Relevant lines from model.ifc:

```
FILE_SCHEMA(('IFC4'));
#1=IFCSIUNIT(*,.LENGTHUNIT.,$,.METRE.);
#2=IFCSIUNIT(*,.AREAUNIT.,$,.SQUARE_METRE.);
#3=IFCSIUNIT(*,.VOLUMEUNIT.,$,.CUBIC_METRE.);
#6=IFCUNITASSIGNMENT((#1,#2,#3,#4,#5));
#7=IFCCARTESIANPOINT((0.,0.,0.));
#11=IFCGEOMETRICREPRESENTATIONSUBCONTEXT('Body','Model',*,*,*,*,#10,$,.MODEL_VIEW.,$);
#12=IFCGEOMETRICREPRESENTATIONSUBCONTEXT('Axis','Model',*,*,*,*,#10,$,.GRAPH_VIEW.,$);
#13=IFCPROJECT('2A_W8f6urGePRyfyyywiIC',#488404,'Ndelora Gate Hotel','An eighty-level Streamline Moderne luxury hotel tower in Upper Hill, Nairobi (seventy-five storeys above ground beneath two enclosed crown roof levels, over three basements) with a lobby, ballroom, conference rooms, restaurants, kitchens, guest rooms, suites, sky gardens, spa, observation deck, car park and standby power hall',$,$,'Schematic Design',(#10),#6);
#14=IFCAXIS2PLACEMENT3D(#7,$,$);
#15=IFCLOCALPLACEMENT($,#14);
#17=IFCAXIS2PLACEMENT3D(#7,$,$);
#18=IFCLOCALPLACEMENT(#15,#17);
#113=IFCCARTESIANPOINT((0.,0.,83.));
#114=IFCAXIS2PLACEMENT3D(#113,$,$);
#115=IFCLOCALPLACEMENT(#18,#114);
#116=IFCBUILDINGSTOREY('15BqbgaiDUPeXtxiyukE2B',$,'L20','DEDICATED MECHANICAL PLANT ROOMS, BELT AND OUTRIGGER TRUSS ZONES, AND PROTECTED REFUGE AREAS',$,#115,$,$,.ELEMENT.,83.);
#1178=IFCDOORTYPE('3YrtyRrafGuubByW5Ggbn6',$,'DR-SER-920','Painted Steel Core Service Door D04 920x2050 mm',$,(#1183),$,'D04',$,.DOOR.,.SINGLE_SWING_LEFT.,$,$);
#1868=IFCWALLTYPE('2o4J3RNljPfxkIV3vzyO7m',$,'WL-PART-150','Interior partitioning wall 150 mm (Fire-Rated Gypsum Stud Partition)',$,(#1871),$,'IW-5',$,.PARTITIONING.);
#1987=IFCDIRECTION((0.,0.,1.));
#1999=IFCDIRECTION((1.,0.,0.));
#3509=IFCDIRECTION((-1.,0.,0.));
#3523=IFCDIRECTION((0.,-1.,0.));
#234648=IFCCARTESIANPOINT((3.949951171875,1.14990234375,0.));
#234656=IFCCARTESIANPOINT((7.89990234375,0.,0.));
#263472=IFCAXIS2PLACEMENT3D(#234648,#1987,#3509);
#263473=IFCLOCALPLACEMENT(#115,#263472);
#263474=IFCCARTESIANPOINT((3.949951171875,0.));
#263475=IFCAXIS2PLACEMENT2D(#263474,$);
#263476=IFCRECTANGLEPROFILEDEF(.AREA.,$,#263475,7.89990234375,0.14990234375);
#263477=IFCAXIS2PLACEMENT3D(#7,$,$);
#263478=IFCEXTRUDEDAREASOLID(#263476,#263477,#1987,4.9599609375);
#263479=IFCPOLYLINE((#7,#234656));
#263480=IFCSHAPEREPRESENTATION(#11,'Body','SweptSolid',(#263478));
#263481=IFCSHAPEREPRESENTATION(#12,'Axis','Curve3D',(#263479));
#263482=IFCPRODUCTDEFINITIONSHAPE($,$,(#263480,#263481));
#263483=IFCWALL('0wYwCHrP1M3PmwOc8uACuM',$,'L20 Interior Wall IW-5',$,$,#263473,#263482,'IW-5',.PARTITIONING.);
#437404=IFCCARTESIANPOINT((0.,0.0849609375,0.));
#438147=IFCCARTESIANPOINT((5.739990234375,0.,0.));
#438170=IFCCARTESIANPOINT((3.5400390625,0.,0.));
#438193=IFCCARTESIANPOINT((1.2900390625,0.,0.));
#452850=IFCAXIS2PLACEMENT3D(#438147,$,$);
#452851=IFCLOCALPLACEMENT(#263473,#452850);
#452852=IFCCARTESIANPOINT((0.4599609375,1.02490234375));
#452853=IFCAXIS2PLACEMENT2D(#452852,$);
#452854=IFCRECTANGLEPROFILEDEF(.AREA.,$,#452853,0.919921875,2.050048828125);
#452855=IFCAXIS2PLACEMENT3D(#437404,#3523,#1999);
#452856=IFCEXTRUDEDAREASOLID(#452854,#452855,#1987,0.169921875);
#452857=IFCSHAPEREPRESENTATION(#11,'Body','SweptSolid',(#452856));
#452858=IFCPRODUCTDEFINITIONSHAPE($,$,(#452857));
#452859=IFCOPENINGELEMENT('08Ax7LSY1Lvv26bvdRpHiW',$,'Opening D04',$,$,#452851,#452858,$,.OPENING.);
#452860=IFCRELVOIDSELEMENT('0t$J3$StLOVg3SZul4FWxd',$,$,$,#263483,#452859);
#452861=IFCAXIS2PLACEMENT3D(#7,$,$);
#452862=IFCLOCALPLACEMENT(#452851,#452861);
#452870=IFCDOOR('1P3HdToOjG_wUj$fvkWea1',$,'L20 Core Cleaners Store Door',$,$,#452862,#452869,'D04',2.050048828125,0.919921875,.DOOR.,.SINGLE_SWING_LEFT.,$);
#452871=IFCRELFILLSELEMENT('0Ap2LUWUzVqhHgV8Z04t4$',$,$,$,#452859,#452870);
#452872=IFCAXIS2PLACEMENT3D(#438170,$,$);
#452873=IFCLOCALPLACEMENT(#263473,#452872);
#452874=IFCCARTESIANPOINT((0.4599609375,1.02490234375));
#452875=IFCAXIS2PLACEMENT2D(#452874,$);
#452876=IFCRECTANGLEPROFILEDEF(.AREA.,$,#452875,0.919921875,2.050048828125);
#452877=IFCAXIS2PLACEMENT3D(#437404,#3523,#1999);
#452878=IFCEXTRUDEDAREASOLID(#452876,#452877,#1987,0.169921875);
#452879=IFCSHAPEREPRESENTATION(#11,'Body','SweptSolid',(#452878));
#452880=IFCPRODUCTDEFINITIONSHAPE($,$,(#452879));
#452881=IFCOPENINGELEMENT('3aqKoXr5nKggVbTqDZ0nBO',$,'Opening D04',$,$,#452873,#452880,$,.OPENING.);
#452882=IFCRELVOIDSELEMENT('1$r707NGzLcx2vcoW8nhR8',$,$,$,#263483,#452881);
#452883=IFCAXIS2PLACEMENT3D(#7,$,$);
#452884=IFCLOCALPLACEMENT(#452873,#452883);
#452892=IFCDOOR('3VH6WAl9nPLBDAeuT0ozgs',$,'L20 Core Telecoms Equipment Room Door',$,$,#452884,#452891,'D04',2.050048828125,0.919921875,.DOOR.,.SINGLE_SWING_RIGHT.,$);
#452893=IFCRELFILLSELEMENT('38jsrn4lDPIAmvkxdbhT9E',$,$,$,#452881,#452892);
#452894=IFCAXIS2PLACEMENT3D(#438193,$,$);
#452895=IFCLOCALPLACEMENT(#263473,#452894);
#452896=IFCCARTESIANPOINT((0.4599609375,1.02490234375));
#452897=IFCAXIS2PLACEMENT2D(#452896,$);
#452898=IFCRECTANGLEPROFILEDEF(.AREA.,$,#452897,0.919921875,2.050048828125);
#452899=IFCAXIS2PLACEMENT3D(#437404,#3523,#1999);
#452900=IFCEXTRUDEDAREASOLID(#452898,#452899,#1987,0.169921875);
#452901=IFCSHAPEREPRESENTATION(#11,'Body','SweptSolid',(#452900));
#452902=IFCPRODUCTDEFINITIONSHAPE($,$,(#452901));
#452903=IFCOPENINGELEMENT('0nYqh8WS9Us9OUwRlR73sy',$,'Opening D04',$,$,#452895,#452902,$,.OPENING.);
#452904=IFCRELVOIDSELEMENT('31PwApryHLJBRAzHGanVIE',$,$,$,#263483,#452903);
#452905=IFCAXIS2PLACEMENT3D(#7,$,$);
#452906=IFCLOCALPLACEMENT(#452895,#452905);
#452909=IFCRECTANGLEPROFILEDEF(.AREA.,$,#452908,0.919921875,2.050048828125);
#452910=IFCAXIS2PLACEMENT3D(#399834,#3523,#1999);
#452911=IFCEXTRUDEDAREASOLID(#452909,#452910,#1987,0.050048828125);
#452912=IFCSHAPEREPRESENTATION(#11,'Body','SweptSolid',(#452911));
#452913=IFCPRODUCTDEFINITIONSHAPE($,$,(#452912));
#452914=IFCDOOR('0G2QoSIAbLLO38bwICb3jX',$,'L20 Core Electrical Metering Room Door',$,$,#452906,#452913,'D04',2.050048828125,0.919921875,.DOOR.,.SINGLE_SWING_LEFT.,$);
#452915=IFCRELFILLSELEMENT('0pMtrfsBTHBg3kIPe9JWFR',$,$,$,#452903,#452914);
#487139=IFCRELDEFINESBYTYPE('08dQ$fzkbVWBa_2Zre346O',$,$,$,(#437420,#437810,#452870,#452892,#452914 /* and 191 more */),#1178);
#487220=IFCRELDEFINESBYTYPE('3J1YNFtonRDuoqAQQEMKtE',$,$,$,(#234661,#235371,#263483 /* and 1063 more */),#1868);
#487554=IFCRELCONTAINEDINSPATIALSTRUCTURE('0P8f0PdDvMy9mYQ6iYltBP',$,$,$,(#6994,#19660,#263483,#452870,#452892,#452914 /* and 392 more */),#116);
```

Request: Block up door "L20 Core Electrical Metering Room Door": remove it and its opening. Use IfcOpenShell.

```python
import ifcopenshell
import ifcopenshell.api.feature
import ifcopenshell.api.root
import ifcopenshell.geom
import ifcopenshell.util.shape

model = ifcopenshell.open("model.ifc")
settings = ifcopenshell.geom.settings()


def volume(element):
    """Net volume in cubic metres, openings subtracted."""
    shape = ifcopenshell.geom.create_shape(settings, element)
    return ifcopenshell.util.shape.get_volume(shape.geometry)


door = model.by_guid("0G2QoSIAbLLO38bwICb3jX")
opening = door.FillsVoids[0].RelatingOpeningElement
wall = opening.VoidsElements[0].RelatingBuildingElement
before = volume(wall)

ifcopenshell.api.root.remove_product(model, product=door)
ifcopenshell.api.feature.remove_feature(model, feature=opening)

after = volume(wall)

print(f"wall volume {before:.3f} -> {after:.3f} m3")

model.write("model-out.ifc")
```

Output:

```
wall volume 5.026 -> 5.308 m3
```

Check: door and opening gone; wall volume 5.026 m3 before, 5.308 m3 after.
